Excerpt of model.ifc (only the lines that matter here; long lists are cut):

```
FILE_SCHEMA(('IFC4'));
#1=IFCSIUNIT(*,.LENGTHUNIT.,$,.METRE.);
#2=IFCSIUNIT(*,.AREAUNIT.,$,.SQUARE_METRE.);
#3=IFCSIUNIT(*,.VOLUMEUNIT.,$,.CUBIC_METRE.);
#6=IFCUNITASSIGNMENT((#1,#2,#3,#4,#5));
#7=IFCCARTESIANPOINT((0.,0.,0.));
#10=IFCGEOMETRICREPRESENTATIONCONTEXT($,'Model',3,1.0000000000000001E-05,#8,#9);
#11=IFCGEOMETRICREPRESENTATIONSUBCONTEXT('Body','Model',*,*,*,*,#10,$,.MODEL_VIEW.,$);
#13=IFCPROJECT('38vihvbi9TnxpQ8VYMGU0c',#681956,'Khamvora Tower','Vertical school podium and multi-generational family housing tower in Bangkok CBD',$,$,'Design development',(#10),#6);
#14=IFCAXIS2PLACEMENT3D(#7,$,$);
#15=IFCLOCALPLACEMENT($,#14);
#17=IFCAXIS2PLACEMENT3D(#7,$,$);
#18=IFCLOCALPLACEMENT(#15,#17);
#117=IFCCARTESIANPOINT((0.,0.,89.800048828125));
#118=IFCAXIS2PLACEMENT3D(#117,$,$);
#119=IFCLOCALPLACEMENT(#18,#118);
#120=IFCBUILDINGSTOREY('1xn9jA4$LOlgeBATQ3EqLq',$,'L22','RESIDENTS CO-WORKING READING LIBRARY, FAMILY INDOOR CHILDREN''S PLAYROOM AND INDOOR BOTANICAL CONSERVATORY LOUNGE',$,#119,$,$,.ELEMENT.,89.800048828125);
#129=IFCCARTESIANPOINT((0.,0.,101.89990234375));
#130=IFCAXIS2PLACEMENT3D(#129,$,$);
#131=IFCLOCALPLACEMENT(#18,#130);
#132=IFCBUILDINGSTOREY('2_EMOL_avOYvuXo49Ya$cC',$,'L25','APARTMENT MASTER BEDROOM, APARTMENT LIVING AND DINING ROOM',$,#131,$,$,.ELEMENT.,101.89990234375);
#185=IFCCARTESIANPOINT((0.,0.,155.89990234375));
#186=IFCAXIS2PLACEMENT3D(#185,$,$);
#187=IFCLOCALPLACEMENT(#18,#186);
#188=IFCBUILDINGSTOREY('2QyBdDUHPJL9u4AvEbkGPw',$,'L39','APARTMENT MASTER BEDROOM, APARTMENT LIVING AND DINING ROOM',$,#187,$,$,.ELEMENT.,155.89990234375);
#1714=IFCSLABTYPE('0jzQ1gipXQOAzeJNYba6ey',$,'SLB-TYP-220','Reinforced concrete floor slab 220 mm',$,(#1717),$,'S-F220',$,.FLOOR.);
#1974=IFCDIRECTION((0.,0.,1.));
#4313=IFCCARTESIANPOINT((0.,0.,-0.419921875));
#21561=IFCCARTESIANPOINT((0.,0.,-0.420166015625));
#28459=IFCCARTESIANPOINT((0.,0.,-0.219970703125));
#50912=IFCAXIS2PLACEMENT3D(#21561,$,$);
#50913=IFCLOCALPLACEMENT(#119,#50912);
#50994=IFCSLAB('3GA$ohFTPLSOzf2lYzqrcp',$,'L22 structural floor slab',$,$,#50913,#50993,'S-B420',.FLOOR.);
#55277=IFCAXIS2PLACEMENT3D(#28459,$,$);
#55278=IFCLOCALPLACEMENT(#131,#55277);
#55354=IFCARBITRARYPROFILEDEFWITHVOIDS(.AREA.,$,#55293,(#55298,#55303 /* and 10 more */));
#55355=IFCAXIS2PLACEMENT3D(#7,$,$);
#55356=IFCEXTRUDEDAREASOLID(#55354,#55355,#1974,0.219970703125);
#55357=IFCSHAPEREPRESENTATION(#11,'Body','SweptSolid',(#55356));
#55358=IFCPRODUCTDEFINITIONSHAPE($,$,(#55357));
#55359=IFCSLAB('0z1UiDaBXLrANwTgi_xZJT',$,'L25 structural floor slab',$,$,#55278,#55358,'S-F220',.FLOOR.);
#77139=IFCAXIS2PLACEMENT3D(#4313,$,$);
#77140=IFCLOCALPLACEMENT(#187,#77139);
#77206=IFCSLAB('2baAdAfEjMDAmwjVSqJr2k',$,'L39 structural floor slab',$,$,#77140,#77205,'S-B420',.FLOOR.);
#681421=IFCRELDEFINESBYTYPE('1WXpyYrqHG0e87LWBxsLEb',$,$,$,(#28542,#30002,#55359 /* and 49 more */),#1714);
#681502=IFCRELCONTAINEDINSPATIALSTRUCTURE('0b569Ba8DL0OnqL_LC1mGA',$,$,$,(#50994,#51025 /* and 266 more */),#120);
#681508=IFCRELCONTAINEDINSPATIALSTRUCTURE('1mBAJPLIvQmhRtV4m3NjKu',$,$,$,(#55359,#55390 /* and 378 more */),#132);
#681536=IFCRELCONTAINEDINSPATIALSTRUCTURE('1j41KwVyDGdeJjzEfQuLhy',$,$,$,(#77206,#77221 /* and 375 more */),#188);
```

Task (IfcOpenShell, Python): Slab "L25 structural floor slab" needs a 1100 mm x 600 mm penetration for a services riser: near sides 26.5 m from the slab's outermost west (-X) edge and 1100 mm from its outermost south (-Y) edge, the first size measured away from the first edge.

```python
import numpy as np
import ifcopenshell
import ifcopenshell.api.feature
import ifcopenshell.api.geometry
import ifcopenshell.api.root
import ifcopenshell.geom
import ifcopenshell.util.placement
import ifcopenshell.util.representation
import ifcopenshell.util.shape
import ifcopenshell.util.unit

model = ifcopenshell.open("model.ifc")
unit_scale = ifcopenshell.util.unit.calculate_unit_scale(model)
settings = ifcopenshell.geom.settings()


def volume(element):
    """Net volume in cubic metres, openings subtracted."""
    shape = ifcopenshell.geom.create_shape(settings, element)
    return ifcopenshell.util.shape.get_volume(shape.geometry)


slab = model.by_guid("0z1UiDaBXLrANwTgi_xZJT")
before = volume(slab)

# Extent in the slab's own axes, in metres. The edges named are its -X and -Y sides.
slab_shape = ifcopenshell.geom.create_shape(settings, slab)
vertices = ifcopenshell.util.shape.get_vertices(slab_shape.geometry)
x_min, y_min, bottom = vertices.min(axis=0)
top = vertices[:, 2].max()

opening = ifcopenshell.api.root.create_entity(model, ifc_class="IfcOpeningElement", name="Services riser opening", predefined_type="OPENING")
context = ifcopenshell.util.representation.get_context(model, "Model", "Body", "MODEL_VIEW")
width, depth = 1.1, 0.6
outline = [(0.0, 0.0), (width, 0.0), (width, depth), (0.0, depth), (0.0, 0.0)]
# Overshoot both faces by 50 mm so the cut is clean.
shape = ifcopenshell.api.geometry.add_slab_representation(
    model, context=context, depth=top - bottom + 0.1, polyline=outline
)
ifcopenshell.api.geometry.assign_representation(model, product=opening, representation=shape)

matrix = ifcopenshell.util.placement.get_local_placement(slab.ObjectPlacement)
matrix[:, 3] = matrix @ np.append(np.array([x_min + 26.5, y_min + 1.1, bottom - 0.05]) / unit_scale, 1.0)
ifcopenshell.api.geometry.edit_object_placement(model, product=opening, matrix=matrix, is_si=False)
ifcopenshell.api.feature.add_feature(model, feature=opening, element=slab)

after = volume(slab)

print(f"slab volume {before:.3f} -> {after:.3f} m3")

model.write("model-out.ifc")
```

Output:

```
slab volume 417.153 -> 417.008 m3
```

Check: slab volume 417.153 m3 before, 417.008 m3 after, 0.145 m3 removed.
